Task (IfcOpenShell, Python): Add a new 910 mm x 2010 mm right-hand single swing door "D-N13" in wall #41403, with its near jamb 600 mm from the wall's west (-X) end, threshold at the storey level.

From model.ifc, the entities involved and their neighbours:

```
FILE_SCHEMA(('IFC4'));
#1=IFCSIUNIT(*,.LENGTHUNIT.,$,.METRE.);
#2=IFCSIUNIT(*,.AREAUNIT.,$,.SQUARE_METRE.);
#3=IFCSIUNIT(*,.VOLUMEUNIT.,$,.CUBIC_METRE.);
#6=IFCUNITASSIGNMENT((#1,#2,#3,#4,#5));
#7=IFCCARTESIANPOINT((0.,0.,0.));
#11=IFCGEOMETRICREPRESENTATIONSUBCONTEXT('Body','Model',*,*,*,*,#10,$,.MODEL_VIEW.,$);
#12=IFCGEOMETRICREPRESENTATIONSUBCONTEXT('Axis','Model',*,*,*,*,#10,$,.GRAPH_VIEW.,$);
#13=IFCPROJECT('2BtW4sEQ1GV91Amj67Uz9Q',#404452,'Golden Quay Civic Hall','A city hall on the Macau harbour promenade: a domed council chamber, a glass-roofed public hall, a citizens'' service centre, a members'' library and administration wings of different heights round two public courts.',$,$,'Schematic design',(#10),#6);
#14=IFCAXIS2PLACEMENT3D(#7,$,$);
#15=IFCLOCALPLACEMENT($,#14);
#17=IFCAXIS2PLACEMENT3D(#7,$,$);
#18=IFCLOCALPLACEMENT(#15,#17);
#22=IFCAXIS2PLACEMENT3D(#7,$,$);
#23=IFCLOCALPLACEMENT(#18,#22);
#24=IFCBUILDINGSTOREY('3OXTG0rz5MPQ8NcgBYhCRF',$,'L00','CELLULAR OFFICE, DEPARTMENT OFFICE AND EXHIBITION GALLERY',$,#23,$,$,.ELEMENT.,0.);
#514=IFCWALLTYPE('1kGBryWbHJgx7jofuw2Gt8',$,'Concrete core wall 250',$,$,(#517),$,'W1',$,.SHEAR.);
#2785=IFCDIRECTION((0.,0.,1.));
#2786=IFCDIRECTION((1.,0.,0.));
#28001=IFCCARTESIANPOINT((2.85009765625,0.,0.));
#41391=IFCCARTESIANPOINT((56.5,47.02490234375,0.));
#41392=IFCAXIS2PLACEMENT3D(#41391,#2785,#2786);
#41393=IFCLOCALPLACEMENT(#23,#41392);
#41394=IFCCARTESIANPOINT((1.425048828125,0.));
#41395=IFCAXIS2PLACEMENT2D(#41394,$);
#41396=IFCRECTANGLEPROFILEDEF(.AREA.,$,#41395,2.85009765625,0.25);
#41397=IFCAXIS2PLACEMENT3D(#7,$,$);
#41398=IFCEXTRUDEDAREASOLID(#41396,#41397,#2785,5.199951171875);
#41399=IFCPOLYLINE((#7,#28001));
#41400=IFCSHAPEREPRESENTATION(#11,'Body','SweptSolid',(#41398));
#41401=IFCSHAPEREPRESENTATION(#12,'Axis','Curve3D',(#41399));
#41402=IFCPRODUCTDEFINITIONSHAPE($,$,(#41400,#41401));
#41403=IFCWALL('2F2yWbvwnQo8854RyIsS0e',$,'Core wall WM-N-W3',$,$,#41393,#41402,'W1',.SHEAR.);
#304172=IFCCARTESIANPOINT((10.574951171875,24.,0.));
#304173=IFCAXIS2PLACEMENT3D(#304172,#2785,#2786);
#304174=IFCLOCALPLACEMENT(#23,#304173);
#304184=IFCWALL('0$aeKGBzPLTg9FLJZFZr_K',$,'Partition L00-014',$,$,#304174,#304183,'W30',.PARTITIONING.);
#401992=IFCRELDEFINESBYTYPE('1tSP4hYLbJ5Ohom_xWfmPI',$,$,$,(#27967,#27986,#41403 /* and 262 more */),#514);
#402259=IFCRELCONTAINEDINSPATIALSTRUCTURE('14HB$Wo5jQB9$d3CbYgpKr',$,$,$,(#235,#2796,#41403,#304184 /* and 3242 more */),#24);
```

```python
import numpy as np
import ifcopenshell
import ifcopenshell.api.feature
import ifcopenshell.api.geometry
import ifcopenshell.api.root
import ifcopenshell.api.spatial
import ifcopenshell.geom
import ifcopenshell.util.element
import ifcopenshell.util.placement
import ifcopenshell.util.representation
import ifcopenshell.util.shape
import ifcopenshell.util.unit

model = ifcopenshell.open("model.ifc")
unit_scale = ifcopenshell.util.unit.calculate_unit_scale(model)
settings = ifcopenshell.geom.settings()


def volume(element):
    """Net volume in cubic metres, openings subtracted."""
    shape = ifcopenshell.geom.create_shape(settings, element)
    return ifcopenshell.util.shape.get_volume(shape.geometry)


wall = model.by_guid("2F2yWbvwnQo8854RyIsS0e")
storey = ifcopenshell.util.element.get_container(wall, ifc_class="IfcBuildingStorey")
context = ifcopenshell.util.representation.get_context(model, "Model", "Body", "MODEL_VIEW")
before = volume(wall)

width, height, from_end, sill = 0.91, 2.01, 0.6, 0.0  # metres

# The wall runs along its own X axis, and the end named is its -X end.
wall_shape = ifcopenshell.geom.create_shape(settings, wall)
x, y, z = ifcopenshell.util.shape.get_vertices(wall_shape.geometry).T
start = x.min() + from_end
face, thickness = float(y.min()), float(y.max() - y.min())
wall_matrix = ifcopenshell.util.placement.get_local_placement(wall.ObjectPlacement)
level = ifcopenshell.util.placement.get_local_placement(storey.ObjectPlacement)[2, 3]


def in_wall(x, y):
    """Placement at x, y metres in the wall's axes, at sill height."""
    matrix = wall_matrix.copy()
    matrix[:, 3] = wall_matrix @ np.array([x / unit_scale, y / unit_scale, 0.0, 1.0])
    matrix[2, 3] = level + sill / unit_scale
    return matrix


# Opening: a box that overshoots both wall faces by 50 mm.
opening = ifcopenshell.api.root.create_entity(model, ifc_class="IfcOpeningElement", predefined_type="OPENING")
box = ifcopenshell.api.geometry.add_wall_representation(
    model, context=context, length=width, height=height, thickness=thickness + 0.1
)
ifcopenshell.api.geometry.assign_representation(model, product=opening, representation=box)
ifcopenshell.api.geometry.edit_object_placement(model, product=opening, matrix=in_wall(start, face - 0.05), is_si=False)
ifcopenshell.api.feature.add_feature(model, feature=opening, element=wall)

door = ifcopenshell.api.root.create_entity(model, ifc_class="IfcDoor", name="D-N13", predefined_type="DOOR")
door.OverallWidth, door.OverallHeight = width / unit_scale, height / unit_scale
door.OperationType = "SINGLE_SWING_RIGHT"
body = ifcopenshell.api.geometry.add_door_representation(
    model,
    context=context,
    overall_width=door.OverallWidth,
    overall_height=door.OverallHeight,
    operation_type="SINGLE_SWING_RIGHT",
    lining_properties={"LiningDepth": thickness / unit_scale, "ThresholdDepth": thickness / unit_scale},
)
ifcopenshell.api.geometry.assign_representation(model, product=door, representation=body)
ifcopenshell.api.spatial.assign_container(model, products=[door], relating_structure=storey)
ifcopenshell.api.feature.add_filling(model, opening=opening, element=door)

# The lining spans the wall, so the door starts at the wall face.
ifcopenshell.api.geometry.edit_object_placement(model, product=door, matrix=in_wall(start, face), is_si=False)

after = volume(wall)

print(f"wall volume {before:.3f} -> {after:.3f} m3")

model.write("model_updated.ifc")
```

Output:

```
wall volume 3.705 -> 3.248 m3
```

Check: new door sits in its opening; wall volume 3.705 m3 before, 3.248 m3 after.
